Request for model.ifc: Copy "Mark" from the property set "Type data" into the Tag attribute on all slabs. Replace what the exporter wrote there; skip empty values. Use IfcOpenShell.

First a look at what the model holds.

```python
import ifcopenshell
import ifcopenshell.util.element

model = ifcopenshell.open("model.ifc")
print(model.schema)
slabs = model.by_type("IfcSlab")
print(len(slabs), "slabs")
for e in slabs[:8]:
    source = ifcopenshell.util.element.get_pset(e, "Type data", "Mark")
    target = e.Tag
    print(e.id(), repr(source), repr(target), sep=" | ")
```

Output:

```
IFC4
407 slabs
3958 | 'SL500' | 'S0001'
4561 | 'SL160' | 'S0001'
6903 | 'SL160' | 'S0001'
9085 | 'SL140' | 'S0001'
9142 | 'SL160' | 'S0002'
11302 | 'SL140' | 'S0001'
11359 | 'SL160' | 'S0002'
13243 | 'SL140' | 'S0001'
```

```python
import ifcopenshell
import ifcopenshell.util.element

model = ifcopenshell.open("model.ifc")

count = 0
for e in model.by_type("IfcSlab"):
    value = ifcopenshell.util.element.get_pset(e, "Type data", "Mark")
    current = e.Tag
    if not value or not value.strip() or current == value:
        continue
    e.Tag = value
    count += 1

print(count, "slabs updated")

model.write("model_edited.ifc")
```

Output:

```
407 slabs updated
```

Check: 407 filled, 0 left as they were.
